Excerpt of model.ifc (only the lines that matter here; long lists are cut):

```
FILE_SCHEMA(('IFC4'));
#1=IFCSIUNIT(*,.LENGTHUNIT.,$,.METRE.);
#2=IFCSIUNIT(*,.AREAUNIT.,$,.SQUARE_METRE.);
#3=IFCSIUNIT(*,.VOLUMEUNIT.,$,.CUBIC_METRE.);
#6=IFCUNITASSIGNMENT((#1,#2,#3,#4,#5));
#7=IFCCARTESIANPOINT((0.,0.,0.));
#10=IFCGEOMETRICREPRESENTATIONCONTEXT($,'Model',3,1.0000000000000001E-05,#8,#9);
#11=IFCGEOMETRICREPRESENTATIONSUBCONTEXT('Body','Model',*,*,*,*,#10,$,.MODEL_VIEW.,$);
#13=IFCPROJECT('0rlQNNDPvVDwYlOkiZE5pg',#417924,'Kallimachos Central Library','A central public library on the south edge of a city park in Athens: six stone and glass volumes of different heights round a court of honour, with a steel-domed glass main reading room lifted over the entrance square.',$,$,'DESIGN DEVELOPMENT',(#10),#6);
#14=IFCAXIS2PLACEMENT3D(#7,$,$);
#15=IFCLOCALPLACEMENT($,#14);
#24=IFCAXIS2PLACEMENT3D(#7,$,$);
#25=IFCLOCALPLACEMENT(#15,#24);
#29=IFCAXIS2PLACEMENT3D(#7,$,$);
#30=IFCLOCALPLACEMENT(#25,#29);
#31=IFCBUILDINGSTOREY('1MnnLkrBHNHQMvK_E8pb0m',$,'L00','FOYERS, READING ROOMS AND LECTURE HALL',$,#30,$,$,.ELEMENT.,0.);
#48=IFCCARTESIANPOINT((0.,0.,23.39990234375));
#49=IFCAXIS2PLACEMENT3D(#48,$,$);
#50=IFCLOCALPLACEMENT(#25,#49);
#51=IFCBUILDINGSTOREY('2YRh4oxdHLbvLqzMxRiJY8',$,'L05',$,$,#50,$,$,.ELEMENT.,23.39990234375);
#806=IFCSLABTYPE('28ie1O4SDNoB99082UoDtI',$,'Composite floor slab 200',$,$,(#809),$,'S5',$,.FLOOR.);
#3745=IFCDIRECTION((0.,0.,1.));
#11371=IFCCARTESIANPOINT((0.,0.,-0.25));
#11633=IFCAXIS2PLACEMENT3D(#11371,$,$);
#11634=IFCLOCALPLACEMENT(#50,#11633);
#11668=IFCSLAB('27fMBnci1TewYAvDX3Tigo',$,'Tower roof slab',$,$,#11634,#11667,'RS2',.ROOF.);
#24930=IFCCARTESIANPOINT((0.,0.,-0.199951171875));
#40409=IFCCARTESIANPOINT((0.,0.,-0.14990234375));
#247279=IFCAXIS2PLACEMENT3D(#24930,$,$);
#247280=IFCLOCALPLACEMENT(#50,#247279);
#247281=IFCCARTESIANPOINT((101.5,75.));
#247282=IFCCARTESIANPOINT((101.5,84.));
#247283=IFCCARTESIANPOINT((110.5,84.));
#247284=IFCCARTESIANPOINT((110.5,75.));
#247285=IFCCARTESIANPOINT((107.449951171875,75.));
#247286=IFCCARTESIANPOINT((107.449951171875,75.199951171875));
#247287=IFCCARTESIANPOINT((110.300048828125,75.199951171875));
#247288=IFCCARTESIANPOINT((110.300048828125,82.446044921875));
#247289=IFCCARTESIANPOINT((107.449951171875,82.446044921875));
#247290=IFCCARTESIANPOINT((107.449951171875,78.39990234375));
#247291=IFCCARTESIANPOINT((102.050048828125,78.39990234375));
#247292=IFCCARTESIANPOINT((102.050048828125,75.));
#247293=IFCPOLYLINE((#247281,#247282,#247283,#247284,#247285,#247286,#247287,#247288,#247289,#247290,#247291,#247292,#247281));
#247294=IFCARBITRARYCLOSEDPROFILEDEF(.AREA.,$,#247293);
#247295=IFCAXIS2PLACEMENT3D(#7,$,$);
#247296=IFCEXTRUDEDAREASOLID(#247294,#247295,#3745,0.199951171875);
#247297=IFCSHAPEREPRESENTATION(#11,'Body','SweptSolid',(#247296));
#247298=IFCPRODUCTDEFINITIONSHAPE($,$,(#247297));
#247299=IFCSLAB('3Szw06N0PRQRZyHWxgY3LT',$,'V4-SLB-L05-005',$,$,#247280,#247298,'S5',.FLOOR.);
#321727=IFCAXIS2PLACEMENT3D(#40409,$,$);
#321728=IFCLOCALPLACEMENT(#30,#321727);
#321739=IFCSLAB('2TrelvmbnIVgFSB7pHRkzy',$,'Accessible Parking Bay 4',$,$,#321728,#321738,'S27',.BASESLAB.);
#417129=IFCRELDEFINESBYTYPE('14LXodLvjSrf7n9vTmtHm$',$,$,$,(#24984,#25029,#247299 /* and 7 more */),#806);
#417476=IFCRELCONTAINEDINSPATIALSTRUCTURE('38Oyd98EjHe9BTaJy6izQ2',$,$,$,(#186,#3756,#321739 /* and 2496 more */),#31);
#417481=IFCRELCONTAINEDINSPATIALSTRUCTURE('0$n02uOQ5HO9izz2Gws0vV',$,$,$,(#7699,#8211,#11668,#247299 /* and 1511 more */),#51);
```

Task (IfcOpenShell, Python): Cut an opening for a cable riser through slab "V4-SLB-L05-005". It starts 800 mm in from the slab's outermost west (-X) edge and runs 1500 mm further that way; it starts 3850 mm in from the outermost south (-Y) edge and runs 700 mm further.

```python
import numpy as np
import ifcopenshell
import ifcopenshell.api.feature
import ifcopenshell.api.geometry
import ifcopenshell.api.root
import ifcopenshell.geom
import ifcopenshell.util.placement
import ifcopenshell.util.representation
import ifcopenshell.util.shape
import ifcopenshell.util.unit

model = ifcopenshell.open("model.ifc")
unit_scale = ifcopenshell.util.unit.calculate_unit_scale(model)
settings = ifcopenshell.geom.settings()


def volume(element):
    """Net volume in cubic metres, openings subtracted."""
    shape = ifcopenshell.geom.create_shape(settings, element)
    return ifcopenshell.util.shape.get_volume(shape.geometry)


slab = model.by_guid("3Szw06N0PRQRZyHWxgY3LT")
before = volume(slab)

# Extent in the slab's own axes, in metres. The edges named are its -X and -Y sides.
slab_shape = ifcopenshell.geom.create_shape(settings, slab)
vertices = ifcopenshell.util.shape.get_vertices(slab_shape.geometry)
x_min, y_min, bottom = vertices.min(axis=0)
top = vertices[:, 2].max()

opening = ifcopenshell.api.root.create_entity(model, ifc_class="IfcOpeningElement", name="Cable riser opening", predefined_type="OPENING")
context = ifcopenshell.util.representation.get_context(model, "Model", "Body", "MODEL_VIEW")
width, depth = 1.5, 0.7
outline = [(0.0, 0.0), (width, 0.0), (width, depth), (0.0, depth), (0.0, 0.0)]
# Overshoot both faces by 50 mm so the cut is clean.
shape = ifcopenshell.api.geometry.add_slab_representation(
    model, context=context, depth=top - bottom + 0.1, polyline=outline
)
ifcopenshell.api.geometry.assign_representation(model, product=opening, representation=shape)

matrix = ifcopenshell.util.placement.get_local_placement(slab.ObjectPlacement)
matrix[:, 3] = matrix @ np.append(np.array([x_min + 0.8, y_min + 3.85, bottom - 0.05]) / unit_scale, 1.0)
ifcopenshell.api.geometry.edit_object_placement(model, product=opening, matrix=matrix, is_si=False)
ifcopenshell.api.feature.add_feature(model, feature=opening, element=slab)

after = volume(slab)

print(f"slab volume {before:.3f} -> {after:.3f} m3")

model.write("model_v2.ifc")
```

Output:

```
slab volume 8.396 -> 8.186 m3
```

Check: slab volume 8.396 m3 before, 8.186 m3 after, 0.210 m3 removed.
